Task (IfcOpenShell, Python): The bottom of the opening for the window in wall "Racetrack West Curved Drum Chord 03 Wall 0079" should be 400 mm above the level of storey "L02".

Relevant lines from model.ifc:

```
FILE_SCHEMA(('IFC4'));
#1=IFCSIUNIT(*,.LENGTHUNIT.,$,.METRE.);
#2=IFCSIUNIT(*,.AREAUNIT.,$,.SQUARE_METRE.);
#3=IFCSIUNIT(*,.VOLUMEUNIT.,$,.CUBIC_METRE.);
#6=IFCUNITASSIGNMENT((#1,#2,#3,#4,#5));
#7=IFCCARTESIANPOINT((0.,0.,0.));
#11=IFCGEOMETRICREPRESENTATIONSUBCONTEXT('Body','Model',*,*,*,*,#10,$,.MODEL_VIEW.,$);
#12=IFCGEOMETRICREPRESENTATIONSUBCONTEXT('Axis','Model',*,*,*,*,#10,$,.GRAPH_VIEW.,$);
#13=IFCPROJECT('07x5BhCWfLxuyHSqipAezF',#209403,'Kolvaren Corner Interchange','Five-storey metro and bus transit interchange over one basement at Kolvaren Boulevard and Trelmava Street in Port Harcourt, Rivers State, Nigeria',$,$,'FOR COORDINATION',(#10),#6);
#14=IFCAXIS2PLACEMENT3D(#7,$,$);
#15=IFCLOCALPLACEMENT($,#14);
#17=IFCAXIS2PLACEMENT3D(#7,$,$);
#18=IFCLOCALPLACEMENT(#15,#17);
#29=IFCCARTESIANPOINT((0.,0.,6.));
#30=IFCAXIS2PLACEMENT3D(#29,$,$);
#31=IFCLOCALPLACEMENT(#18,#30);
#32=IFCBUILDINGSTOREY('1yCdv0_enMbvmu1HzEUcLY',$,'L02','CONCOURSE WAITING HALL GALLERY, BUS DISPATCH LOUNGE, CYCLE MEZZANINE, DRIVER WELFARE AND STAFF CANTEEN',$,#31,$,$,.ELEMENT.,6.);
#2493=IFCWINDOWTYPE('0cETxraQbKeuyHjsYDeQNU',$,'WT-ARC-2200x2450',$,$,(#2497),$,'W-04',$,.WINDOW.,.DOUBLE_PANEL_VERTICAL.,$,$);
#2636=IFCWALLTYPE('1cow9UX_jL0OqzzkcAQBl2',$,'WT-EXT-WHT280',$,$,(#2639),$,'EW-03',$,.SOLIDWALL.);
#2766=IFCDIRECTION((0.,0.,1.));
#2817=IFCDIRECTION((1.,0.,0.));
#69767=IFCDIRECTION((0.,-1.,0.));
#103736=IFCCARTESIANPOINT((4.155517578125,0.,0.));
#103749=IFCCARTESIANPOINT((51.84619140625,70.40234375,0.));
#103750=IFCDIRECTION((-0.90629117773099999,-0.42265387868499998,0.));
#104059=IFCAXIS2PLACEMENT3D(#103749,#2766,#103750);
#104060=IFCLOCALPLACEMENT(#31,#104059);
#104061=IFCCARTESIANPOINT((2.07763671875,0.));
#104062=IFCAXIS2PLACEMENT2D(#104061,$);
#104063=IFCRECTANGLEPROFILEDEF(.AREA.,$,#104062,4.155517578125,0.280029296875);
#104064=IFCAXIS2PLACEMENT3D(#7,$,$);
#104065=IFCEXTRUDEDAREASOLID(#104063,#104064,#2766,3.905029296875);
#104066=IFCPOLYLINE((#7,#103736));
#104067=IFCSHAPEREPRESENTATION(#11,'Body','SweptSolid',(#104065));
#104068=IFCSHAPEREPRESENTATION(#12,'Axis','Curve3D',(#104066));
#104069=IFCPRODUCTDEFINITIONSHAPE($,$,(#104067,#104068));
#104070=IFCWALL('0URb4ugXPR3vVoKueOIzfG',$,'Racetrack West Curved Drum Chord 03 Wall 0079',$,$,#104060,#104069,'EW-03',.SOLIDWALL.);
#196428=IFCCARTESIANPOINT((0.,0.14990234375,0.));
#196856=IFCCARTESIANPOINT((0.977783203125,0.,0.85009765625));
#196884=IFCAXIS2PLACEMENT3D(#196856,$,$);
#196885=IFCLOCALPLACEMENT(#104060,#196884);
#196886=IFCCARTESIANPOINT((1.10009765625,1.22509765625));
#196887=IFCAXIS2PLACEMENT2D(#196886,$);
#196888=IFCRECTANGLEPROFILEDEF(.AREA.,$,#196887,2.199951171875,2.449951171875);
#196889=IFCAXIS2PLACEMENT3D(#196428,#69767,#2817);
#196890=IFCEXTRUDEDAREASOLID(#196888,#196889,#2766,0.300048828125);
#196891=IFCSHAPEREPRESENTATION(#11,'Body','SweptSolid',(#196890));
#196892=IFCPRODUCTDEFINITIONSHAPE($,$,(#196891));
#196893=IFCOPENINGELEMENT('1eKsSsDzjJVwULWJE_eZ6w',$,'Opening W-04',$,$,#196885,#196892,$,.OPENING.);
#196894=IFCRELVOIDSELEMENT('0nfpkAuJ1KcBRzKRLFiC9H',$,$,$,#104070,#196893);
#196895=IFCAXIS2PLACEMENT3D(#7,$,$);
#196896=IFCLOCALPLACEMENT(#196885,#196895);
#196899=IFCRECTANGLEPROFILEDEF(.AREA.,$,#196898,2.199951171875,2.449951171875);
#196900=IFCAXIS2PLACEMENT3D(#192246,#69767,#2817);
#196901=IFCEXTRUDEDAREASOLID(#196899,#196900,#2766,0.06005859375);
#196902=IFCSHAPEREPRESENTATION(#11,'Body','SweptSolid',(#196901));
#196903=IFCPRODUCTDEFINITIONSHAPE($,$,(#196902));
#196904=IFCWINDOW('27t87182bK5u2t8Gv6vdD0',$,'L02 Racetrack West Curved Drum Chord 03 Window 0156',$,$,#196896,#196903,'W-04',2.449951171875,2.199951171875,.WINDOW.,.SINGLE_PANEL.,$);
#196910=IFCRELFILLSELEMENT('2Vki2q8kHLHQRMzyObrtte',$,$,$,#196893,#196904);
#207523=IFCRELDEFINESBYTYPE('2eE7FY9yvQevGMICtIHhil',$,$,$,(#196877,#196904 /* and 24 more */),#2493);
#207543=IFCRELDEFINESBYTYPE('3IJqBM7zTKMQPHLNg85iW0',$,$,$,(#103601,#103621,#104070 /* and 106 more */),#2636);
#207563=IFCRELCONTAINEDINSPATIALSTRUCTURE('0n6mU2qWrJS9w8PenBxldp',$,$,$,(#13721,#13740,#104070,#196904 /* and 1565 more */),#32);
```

```python
import numpy as np
import ifcopenshell
import ifcopenshell.api.geometry
import ifcopenshell.geom
import ifcopenshell.util.element
import ifcopenshell.util.placement
import ifcopenshell.util.shape
import ifcopenshell.util.unit

model = ifcopenshell.open("model.ifc")
unit_scale = ifcopenshell.util.unit.calculate_unit_scale(model)

window = model.by_guid("27t87182bK5u2t8Gv6vdD0")
opening = window.FillsVoids[0].RelatingOpeningElement
storey = ifcopenshell.util.element.get_container(window, ifc_class="IfcBuildingStorey")
level = ifcopenshell.util.placement.get_local_placement(storey.ObjectPlacement)[2, 3]

# The opening's origin need not be at the sill, so measure its lowest point.
shape = ifcopenshell.geom.create_shape(ifcopenshell.geom.settings(), opening)
bottom = ifcopenshell.util.shape.get_shape_bottom_elevation(shape, shape.geometry) / unit_scale
dz = level + 0.4 - bottom

shift = np.array([0.0, 0.0, dz])
# The window is placed relative to its opening, so it follows when the opening moves.
matrix = ifcopenshell.util.placement.get_local_placement(opening.ObjectPlacement)
matrix[:3, 3] += shift
ifcopenshell.api.geometry.edit_object_placement(
    model, product=opening, matrix=matrix, is_si=False, should_transform_children=True
)

print(f"moved by {dz * unit_scale:+.3f} m")

model.write("model_edited.ifc")
```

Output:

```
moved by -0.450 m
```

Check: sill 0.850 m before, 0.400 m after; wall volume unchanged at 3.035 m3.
